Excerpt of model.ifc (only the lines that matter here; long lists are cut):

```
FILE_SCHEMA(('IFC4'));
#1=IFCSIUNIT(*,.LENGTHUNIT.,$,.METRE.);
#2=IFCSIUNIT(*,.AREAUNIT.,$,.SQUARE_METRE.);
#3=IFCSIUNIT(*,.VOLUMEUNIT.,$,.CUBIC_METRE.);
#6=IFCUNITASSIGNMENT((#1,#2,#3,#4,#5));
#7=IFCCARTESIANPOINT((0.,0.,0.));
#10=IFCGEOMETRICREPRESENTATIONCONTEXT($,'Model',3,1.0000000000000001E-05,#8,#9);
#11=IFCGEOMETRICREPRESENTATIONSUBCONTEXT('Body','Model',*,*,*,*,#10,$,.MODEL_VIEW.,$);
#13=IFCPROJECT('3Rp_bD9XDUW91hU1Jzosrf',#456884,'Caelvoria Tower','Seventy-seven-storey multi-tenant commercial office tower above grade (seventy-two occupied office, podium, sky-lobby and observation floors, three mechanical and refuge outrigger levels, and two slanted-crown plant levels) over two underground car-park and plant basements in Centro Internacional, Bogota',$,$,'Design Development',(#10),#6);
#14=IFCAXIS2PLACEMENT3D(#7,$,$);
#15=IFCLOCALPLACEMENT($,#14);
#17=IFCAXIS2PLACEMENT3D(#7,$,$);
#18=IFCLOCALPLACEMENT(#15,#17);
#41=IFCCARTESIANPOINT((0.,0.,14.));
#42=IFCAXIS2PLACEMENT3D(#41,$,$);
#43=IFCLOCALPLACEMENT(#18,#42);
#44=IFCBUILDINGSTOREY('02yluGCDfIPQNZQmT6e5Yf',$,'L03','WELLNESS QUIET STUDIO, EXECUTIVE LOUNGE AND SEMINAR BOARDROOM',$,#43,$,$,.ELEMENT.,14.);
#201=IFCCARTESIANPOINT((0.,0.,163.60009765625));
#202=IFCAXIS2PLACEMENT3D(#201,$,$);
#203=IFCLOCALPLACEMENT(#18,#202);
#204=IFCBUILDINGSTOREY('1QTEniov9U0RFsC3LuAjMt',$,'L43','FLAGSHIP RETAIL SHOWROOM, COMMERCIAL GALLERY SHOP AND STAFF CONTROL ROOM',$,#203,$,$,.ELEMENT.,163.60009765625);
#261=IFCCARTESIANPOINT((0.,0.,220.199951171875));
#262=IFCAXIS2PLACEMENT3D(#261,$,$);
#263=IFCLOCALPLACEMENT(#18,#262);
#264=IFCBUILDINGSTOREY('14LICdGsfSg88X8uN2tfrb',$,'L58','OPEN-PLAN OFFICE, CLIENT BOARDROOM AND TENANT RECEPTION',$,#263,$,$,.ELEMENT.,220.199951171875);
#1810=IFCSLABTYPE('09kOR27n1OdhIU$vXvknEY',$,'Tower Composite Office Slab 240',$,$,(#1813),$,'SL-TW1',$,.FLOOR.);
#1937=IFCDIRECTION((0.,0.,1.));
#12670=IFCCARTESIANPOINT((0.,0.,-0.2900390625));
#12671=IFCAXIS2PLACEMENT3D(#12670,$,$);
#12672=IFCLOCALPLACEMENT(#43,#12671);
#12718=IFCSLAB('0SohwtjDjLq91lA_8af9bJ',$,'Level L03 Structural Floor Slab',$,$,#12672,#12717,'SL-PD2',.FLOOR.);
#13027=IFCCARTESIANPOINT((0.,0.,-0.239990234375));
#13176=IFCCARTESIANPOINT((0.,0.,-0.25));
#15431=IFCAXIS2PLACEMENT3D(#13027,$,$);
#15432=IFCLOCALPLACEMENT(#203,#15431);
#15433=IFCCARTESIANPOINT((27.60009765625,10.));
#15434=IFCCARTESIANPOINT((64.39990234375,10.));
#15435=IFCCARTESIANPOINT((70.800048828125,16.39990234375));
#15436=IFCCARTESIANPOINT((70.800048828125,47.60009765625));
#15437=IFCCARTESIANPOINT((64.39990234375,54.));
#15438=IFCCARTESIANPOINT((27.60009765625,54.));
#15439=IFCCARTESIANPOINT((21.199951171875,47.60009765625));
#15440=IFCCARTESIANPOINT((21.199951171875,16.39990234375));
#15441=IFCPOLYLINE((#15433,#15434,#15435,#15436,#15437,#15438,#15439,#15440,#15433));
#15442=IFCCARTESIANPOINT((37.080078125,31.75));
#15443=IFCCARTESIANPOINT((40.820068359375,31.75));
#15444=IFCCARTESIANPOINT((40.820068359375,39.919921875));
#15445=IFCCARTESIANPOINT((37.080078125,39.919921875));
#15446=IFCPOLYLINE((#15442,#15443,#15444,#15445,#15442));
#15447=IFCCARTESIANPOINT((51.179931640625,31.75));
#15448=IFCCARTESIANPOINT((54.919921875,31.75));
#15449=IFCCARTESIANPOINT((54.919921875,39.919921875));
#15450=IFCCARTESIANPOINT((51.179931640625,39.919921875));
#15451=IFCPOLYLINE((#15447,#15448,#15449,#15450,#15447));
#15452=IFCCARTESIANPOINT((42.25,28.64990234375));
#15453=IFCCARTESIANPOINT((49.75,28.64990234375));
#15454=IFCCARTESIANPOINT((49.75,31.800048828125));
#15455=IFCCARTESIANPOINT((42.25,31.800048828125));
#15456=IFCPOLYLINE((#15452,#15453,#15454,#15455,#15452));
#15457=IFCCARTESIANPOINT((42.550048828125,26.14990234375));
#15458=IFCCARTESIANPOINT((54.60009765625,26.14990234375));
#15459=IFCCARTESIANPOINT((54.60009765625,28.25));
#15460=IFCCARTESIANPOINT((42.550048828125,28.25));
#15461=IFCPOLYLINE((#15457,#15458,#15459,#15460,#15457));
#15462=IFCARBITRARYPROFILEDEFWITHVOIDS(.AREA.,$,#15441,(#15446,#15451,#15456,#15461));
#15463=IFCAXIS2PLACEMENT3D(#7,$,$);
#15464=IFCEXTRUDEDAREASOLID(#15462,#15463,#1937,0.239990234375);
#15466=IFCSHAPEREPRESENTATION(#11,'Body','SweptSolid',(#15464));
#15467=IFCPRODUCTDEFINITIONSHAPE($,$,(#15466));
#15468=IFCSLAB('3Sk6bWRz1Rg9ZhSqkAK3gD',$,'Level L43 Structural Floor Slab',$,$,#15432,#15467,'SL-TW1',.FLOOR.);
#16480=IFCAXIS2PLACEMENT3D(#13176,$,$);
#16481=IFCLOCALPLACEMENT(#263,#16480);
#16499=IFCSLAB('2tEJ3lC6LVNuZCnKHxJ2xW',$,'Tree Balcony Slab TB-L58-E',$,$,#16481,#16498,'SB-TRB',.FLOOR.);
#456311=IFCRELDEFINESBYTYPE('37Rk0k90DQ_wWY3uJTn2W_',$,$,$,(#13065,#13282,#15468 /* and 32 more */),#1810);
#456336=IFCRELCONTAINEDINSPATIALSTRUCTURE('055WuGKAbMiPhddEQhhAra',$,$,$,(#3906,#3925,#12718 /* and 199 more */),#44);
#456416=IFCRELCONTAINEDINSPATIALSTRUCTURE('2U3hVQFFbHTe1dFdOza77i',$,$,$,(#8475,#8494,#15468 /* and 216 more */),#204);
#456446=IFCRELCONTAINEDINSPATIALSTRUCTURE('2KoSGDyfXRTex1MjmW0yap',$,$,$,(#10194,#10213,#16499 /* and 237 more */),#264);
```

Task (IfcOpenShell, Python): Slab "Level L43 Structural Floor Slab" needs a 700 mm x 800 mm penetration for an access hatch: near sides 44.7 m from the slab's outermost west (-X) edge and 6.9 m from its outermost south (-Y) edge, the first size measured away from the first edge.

```python
import numpy as np
import ifcopenshell
import ifcopenshell.api.feature
import ifcopenshell.api.geometry
import ifcopenshell.api.root
import ifcopenshell.geom
import ifcopenshell.util.placement
import ifcopenshell.util.representation
import ifcopenshell.util.shape
import ifcopenshell.util.unit

model = ifcopenshell.open("model.ifc")
unit_scale = ifcopenshell.util.unit.calculate_unit_scale(model)
settings = ifcopenshell.geom.settings()


def volume(element):
    """Net volume in cubic metres, openings subtracted."""
    shape = ifcopenshell.geom.create_shape(settings, element)
    return ifcopenshell.util.shape.get_volume(shape.geometry)


slab = model.by_id(15468)
before = volume(slab)

# Extent in the slab's own axes, in metres. The edges named are its -X and -Y sides.
slab_shape = ifcopenshell.geom.create_shape(settings, slab)
vertices = ifcopenshell.util.shape.get_vertices(slab_shape.geometry)
x_min, y_min, bottom = vertices.min(axis=0)
top = vertices[:, 2].max()

opening = ifcopenshell.api.root.create_entity(model, ifc_class="IfcOpeningElement", name="Access hatch opening", predefined_type="OPENING")
context = ifcopenshell.util.representation.get_context(model, "Model", "Body", "MODEL_VIEW")
width, depth = 0.7, 0.8
outline = [(0.0, 0.0), (width, 0.0), (width, depth), (0.0, depth), (0.0, 0.0)]
# Overshoot both faces by 50 mm so the cut is clean.
shape = ifcopenshell.api.geometry.add_slab_representation(
    model, context=context, depth=top - bottom + 0.1, polyline=outline
)
ifcopenshell.api.geometry.assign_representation(model, product=opening, representation=shape)

matrix = ifcopenshell.util.placement.get_local_placement(slab.ObjectPlacement)
matrix[:, 3] = matrix @ np.append(np.array([x_min + 44.7, y_min + 6.9, bottom - 0.05]) / unit_scale, 1.0)
ifcopenshell.api.geometry.edit_object_placement(model, product=opening, matrix=matrix, is_si=False)
ifcopenshell.api.feature.add_feature(model, feature=opening, element=slab)

after = volume(slab)

print(f"slab volume {before:.3f} -> {after:.3f} m3")

model.write("model-out.ifc")
```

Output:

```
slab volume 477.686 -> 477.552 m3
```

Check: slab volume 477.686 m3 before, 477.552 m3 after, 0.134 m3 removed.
